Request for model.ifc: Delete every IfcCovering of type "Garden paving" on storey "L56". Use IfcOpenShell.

First a look at what the model holds.

```python
import ifcopenshell
import ifcopenshell.util.element

model = ifcopenshell.open("model.ifc")
print(model.schema)
storey = next(s for s in model.by_type("IfcBuildingStorey") if s.Name == "L56")
coverings = [e for e in ifcopenshell.util.element.get_decomposition(storey) if e.is_a("IfcCovering")]
seen = {}
for e in coverings:
    element_type = ifcopenshell.util.element.get_type(e)
    name = element_type.Name if element_type not in (None, e) else None
    seen[name] = seen.get(name, 0) + 1
for name, count in sorted(seen.items(), key=str):
    print(count, "x", name)
```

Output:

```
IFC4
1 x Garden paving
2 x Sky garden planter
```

```python
import ifcopenshell
import ifcopenshell.api.root
import ifcopenshell.util.element

model = ifcopenshell.open("model.ifc")

storey = next(s for s in model.by_type("IfcBuildingStorey") if s.Name == "L56")
coverings = [e for e in ifcopenshell.util.element.get_decomposition(storey) if e.is_a("IfcCovering")]
targets = [e for e in coverings if (t := ifcopenshell.util.element.get_type(e)) not in (None, e) and t.Name == "Garden paving"]

for e in targets:
    ifcopenshell.api.root.remove_product(model, product=e)
print(len(targets), "removed")

model.write("model_rev.ifc")
```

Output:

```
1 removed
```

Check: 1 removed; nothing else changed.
